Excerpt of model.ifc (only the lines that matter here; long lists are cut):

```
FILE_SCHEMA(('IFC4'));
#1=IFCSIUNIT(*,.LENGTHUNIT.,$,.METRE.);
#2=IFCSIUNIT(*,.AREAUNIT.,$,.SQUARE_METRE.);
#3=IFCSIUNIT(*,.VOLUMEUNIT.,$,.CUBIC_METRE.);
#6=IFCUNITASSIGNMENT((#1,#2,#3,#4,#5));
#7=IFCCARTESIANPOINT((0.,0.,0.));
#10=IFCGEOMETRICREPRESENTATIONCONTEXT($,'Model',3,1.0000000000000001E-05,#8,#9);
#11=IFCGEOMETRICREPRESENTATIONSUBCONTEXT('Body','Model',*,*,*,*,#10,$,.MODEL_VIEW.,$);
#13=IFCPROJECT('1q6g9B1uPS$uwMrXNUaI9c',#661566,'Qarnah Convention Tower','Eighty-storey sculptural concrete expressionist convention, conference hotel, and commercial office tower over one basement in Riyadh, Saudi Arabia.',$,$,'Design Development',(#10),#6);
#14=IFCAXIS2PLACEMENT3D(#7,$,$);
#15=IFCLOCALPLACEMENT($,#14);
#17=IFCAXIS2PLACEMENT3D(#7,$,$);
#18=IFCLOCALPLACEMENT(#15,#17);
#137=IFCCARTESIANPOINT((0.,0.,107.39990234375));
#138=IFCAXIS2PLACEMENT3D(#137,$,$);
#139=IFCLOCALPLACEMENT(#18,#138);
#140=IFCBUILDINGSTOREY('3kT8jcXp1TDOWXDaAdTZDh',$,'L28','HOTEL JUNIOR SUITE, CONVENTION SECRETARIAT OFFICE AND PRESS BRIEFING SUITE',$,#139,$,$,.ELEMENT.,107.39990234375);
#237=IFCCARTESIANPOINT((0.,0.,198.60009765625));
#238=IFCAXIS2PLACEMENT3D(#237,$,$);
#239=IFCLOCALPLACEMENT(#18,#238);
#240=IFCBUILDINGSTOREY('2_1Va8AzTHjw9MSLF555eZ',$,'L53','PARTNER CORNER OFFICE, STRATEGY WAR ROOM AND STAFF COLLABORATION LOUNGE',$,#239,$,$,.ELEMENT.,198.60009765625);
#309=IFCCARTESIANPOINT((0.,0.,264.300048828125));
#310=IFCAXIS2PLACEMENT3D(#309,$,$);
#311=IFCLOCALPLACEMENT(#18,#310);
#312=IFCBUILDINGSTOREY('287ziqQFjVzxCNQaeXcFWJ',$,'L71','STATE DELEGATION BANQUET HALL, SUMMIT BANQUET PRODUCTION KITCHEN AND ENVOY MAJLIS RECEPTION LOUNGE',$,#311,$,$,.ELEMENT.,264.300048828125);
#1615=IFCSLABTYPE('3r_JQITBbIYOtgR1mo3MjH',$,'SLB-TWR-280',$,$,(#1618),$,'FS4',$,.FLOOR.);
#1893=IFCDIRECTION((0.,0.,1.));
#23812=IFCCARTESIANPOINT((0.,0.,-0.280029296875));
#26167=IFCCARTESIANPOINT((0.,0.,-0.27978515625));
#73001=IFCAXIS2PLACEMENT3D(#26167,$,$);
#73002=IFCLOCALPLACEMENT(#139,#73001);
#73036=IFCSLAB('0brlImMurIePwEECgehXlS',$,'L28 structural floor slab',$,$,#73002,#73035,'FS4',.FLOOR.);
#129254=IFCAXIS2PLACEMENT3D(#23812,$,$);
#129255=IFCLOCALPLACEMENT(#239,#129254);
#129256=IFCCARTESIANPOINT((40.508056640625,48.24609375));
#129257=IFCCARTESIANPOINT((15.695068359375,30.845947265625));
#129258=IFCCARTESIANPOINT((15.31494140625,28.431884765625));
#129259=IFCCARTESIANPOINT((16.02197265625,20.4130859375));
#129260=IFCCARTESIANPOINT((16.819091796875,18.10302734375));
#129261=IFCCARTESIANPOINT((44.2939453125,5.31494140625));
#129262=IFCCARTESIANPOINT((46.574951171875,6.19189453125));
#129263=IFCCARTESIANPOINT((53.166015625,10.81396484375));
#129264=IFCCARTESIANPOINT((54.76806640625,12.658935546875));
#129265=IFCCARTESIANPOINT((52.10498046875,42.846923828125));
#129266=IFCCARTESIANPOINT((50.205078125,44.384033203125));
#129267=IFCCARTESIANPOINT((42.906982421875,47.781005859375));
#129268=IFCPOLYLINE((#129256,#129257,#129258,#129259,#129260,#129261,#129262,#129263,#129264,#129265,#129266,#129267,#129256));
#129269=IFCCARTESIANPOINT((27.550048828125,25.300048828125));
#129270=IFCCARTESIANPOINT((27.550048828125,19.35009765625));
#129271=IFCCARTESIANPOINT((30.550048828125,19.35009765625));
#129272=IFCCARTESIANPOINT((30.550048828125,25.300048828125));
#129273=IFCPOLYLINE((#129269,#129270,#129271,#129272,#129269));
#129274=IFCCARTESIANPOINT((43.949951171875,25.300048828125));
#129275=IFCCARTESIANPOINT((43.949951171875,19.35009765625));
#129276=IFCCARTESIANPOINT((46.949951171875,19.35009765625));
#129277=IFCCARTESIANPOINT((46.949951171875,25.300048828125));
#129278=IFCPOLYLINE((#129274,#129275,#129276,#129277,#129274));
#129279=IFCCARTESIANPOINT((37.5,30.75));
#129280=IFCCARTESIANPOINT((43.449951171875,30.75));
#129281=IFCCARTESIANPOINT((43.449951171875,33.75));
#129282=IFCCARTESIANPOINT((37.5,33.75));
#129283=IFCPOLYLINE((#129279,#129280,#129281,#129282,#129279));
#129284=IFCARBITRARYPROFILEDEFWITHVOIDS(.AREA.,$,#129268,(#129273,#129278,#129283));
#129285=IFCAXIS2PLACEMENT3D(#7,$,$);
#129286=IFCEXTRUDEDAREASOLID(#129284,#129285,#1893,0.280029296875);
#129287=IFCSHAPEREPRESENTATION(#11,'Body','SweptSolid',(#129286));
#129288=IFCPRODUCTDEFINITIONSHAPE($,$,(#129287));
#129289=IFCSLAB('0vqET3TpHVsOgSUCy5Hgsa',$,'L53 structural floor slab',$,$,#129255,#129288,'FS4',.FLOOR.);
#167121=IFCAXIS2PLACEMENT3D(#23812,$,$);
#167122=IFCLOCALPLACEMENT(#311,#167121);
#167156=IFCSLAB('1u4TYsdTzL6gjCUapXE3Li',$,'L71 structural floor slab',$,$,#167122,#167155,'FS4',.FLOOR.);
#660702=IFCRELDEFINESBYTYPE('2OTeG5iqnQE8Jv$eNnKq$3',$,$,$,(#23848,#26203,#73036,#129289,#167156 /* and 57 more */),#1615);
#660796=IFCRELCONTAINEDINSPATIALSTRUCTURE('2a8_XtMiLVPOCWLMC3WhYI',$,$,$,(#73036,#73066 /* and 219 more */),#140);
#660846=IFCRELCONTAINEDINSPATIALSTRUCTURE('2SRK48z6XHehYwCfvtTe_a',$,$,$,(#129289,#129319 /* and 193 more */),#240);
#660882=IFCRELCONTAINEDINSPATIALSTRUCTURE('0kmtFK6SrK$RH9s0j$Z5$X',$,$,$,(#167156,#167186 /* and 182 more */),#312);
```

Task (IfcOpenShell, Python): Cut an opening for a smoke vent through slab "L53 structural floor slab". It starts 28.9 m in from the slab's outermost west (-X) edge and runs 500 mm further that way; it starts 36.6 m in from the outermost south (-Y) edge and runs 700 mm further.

```python
import numpy as np
import ifcopenshell
import ifcopenshell.api.feature
import ifcopenshell.api.geometry
import ifcopenshell.api.root
import ifcopenshell.geom
import ifcopenshell.util.placement
import ifcopenshell.util.representation
import ifcopenshell.util.shape
import ifcopenshell.util.unit

model = ifcopenshell.open("model.ifc")
unit_scale = ifcopenshell.util.unit.calculate_unit_scale(model)
settings = ifcopenshell.geom.settings()


def volume(element):
    """Net volume in cubic metres, openings subtracted."""
    shape = ifcopenshell.geom.create_shape(settings, element)
    return ifcopenshell.util.shape.get_volume(shape.geometry)


slab = model.by_guid("0vqET3TpHVsOgSUCy5Hgsa")
before = volume(slab)

# Extent in the slab's own axes, in metres. The edges named are its -X and -Y sides.
slab_shape = ifcopenshell.geom.create_shape(settings, slab)
vertices = ifcopenshell.util.shape.get_vertices(slab_shape.geometry)
x_min, y_min, bottom = vertices.min(axis=0)
top = vertices[:, 2].max()

opening = ifcopenshell.api.root.create_entity(model, ifc_class="IfcOpeningElement", name="Smoke vent opening", predefined_type="OPENING")
context = ifcopenshell.util.representation.get_context(model, "Model", "Body", "MODEL_VIEW")
width, depth = 0.5, 0.7
outline = [(0.0, 0.0), (width, 0.0), (width, depth), (0.0, depth), (0.0, 0.0)]
# Overshoot both faces by 50 mm so the cut is clean.
shape = ifcopenshell.api.geometry.add_slab_representation(
    model, context=context, depth=top - bottom + 0.1, polyline=outline
)
ifcopenshell.api.geometry.assign_representation(model, product=opening, representation=shape)

matrix = ifcopenshell.util.placement.get_local_placement(slab.ObjectPlacement)
matrix[:, 3] = matrix @ np.append(np.array([x_min + 28.9, y_min + 36.6, bottom - 0.05]) / unit_scale, 1.0)
ifcopenshell.api.geometry.edit_object_placement(model, product=opening, matrix=matrix, is_si=False)
ifcopenshell.api.feature.add_feature(model, feature=opening, element=slab)

after = volume(slab)

print(f"slab volume {before:.3f} -> {after:.3f} m3")

model.write("model_v2.ifc")
```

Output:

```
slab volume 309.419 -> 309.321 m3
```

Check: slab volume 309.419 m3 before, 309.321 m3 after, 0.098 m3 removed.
